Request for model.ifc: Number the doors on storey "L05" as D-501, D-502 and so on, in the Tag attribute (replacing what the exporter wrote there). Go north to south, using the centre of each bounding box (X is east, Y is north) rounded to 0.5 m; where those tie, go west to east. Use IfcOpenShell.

First a look at what the model holds.

```python
import ifcopenshell
import ifcopenshell.util.element
import ifcopenshell.util.placement

model = ifcopenshell.open("model.ifc")
print(model.schema)
storey = next(s for s in model.by_type("IfcBuildingStorey") if s.Name == "L05")
doors = [e for e in ifcopenshell.util.element.get_decomposition(storey) if e.is_a("IfcDoor")]
for e in sorted(doors, key=lambda e: e.id()):
    origin = ifcopenshell.util.placement.get_local_placement(e.ObjectPlacement)[:3, 3]
    print(e.id(), e.Tag, e.Name, origin.round(2) + 0.0, sep=" | ")
```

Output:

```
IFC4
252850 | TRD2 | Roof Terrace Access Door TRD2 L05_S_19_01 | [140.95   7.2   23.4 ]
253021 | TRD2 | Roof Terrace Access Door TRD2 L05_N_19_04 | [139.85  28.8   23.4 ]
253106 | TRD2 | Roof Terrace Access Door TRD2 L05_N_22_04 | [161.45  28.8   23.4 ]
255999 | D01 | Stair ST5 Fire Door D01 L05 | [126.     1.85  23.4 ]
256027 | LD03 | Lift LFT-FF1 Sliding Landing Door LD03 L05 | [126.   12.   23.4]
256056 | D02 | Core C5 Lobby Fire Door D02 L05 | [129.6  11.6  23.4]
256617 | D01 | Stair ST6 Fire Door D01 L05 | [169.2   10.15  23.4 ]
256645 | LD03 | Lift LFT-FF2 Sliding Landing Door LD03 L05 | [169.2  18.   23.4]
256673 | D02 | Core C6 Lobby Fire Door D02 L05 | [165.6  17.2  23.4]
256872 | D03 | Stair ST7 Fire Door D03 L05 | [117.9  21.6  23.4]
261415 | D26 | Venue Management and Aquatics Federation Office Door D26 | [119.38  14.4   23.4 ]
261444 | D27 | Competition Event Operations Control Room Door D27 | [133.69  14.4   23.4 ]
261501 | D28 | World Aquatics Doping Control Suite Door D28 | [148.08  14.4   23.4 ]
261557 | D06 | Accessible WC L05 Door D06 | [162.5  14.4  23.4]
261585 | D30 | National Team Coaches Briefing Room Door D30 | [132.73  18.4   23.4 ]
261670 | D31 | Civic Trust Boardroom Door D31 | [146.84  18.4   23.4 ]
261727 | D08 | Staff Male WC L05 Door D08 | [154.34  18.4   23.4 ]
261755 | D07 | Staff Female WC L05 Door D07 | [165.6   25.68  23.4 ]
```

```python
import ifcopenshell
import ifcopenshell.geom
import ifcopenshell.util.element
import ifcopenshell.util.shape

model = ifcopenshell.open("model.ifc")
settings = ifcopenshell.geom.settings()
settings.set("use-world-coords", True)


def centre(element):
    shape = ifcopenshell.geom.create_shape(settings, element)
    return ifcopenshell.util.shape.get_bbox_centroid(shape.geometry)


storey = next(s for s in model.by_type("IfcBuildingStorey") if s.Name == "L05")
doors = [e for e in ifcopenshell.util.element.get_decomposition(storey) if e.is_a("IfcDoor")]

# Insertion points can sit at a corner or the storey origin, so sort by the geometry (in metres).
centres = {e: centre(e) for e in doors}
doors.sort(key=lambda e: (-round(centres[e][1] / 0.5), centres[e][0]))

for i, e in enumerate(doors, start=1):
    number = f"D-5{i:02d}"
    e.Tag = number
    print(e.id(), number)

model.write("model_rev.ifc")
```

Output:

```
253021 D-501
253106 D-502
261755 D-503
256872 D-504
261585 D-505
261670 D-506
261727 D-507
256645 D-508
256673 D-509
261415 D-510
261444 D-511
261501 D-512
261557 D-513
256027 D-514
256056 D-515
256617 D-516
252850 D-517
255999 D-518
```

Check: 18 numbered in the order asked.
